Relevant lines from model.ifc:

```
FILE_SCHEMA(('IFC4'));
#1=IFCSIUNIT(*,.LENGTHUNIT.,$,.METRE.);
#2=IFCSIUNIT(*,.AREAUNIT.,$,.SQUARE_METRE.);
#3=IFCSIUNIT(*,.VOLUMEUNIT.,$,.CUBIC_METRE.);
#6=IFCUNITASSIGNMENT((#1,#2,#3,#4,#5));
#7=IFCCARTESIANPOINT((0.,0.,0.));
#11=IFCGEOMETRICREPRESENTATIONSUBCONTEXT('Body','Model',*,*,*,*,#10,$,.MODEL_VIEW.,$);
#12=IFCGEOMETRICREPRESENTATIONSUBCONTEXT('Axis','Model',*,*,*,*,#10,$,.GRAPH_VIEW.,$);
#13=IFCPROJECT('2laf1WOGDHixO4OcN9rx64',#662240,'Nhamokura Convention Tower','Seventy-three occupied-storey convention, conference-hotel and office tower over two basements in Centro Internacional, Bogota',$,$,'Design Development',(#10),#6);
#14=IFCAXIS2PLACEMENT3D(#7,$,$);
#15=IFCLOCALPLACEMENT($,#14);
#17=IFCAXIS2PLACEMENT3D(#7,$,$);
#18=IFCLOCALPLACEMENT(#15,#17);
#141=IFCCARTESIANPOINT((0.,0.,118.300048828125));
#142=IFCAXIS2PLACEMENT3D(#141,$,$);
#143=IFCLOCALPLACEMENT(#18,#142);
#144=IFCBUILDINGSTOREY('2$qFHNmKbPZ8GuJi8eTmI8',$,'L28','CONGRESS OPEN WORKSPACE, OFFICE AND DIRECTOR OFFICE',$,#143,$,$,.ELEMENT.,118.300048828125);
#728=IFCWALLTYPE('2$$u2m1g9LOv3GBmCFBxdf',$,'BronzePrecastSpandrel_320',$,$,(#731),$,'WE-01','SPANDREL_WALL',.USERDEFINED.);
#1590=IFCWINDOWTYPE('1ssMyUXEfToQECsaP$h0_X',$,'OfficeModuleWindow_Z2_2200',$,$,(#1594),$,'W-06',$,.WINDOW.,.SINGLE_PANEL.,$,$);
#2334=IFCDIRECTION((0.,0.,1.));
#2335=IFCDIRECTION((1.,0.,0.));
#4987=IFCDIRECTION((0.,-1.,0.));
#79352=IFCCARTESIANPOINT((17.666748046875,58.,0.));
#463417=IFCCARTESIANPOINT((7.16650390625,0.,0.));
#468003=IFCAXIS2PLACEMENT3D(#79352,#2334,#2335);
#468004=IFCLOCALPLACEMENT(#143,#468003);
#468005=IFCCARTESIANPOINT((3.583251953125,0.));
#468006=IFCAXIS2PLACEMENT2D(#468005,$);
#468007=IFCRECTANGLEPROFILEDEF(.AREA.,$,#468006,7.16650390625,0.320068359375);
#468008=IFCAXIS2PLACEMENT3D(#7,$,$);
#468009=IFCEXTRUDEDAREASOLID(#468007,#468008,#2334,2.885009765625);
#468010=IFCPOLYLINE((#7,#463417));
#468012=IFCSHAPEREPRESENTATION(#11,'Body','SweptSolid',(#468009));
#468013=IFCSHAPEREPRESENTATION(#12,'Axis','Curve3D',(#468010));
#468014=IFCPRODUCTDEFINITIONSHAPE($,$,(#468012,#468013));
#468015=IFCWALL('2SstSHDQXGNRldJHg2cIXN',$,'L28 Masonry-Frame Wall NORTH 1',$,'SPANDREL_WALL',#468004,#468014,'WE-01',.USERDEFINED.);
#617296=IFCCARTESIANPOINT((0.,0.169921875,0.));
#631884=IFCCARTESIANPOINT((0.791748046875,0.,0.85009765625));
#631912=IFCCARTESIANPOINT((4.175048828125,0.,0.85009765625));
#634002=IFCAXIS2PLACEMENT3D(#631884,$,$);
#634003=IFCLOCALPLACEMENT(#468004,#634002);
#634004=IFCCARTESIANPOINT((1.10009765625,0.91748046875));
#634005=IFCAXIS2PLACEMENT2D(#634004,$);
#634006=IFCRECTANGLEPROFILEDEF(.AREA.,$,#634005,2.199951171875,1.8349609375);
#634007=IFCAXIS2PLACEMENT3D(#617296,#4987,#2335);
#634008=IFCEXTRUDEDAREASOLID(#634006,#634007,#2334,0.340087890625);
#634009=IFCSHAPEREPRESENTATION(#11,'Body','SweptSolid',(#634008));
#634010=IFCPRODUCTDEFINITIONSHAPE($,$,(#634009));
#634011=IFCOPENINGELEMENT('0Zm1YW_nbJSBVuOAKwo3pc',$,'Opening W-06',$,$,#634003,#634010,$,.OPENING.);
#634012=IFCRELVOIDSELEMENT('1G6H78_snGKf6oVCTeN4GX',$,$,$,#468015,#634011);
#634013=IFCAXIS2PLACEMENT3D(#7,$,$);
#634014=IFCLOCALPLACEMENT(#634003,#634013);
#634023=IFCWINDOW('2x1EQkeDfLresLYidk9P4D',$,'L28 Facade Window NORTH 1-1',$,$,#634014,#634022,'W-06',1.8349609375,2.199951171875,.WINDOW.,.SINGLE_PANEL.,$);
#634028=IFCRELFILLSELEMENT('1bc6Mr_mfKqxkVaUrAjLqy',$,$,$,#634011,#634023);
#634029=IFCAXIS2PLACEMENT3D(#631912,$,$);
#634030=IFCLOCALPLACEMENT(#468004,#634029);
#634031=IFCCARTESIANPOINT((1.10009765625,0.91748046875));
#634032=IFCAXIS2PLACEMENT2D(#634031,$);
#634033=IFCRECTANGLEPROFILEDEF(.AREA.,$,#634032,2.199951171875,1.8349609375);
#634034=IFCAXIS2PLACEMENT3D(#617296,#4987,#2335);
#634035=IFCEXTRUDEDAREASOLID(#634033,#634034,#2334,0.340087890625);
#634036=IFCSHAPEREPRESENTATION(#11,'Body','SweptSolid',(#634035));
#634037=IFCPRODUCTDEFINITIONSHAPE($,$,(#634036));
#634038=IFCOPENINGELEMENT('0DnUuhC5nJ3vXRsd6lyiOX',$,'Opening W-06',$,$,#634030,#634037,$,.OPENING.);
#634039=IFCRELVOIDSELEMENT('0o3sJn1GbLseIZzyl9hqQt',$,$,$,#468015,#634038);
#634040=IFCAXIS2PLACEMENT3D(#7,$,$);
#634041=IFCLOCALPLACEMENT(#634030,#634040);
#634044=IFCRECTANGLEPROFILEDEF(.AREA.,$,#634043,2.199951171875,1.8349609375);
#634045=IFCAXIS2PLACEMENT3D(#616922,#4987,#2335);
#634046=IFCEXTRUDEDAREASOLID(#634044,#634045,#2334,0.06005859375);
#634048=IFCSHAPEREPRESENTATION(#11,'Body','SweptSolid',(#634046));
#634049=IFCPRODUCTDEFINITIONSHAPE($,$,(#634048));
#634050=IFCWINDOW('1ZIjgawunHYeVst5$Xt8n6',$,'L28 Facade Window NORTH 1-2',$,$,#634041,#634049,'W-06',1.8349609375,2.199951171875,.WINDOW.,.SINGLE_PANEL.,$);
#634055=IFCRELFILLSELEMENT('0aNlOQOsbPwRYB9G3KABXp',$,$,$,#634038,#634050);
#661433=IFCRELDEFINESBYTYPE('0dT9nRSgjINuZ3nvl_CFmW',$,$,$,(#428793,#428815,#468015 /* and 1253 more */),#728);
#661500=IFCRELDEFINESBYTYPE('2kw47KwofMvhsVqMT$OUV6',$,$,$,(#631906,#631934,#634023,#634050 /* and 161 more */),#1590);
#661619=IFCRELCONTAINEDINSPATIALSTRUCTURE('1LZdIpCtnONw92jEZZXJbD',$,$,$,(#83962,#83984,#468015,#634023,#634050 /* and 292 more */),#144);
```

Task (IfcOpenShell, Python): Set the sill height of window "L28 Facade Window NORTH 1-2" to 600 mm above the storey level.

```python
import numpy as np
import ifcopenshell
import ifcopenshell.api.geometry
import ifcopenshell.geom
import ifcopenshell.util.element
import ifcopenshell.util.placement
import ifcopenshell.util.shape
import ifcopenshell.util.unit

model = ifcopenshell.open("model.ifc")
unit_scale = ifcopenshell.util.unit.calculate_unit_scale(model)

window = model.by_id(634050)
opening = window.FillsVoids[0].RelatingOpeningElement
storey = ifcopenshell.util.element.get_container(window, ifc_class="IfcBuildingStorey")
level = ifcopenshell.util.placement.get_local_placement(storey.ObjectPlacement)[2, 3]

# The opening's origin need not be at the sill, so measure its lowest point.
shape = ifcopenshell.geom.create_shape(ifcopenshell.geom.settings(), opening)
bottom = ifcopenshell.util.shape.get_shape_bottom_elevation(shape, shape.geometry) / unit_scale
dz = level + 0.6 / unit_scale - bottom

shift = np.array([0.0, 0.0, dz])
# The window is placed relative to its opening, so it follows when the opening moves.
matrix = ifcopenshell.util.placement.get_local_placement(opening.ObjectPlacement)
matrix[:3, 3] += shift
ifcopenshell.api.geometry.edit_object_placement(
    model, product=opening, matrix=matrix, is_si=False, should_transform_children=True
)

print(f"moved by {dz * unit_scale:+.3f} m")

model.write("model-out.ifc")
```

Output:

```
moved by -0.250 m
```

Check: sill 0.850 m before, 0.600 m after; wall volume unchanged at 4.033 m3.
